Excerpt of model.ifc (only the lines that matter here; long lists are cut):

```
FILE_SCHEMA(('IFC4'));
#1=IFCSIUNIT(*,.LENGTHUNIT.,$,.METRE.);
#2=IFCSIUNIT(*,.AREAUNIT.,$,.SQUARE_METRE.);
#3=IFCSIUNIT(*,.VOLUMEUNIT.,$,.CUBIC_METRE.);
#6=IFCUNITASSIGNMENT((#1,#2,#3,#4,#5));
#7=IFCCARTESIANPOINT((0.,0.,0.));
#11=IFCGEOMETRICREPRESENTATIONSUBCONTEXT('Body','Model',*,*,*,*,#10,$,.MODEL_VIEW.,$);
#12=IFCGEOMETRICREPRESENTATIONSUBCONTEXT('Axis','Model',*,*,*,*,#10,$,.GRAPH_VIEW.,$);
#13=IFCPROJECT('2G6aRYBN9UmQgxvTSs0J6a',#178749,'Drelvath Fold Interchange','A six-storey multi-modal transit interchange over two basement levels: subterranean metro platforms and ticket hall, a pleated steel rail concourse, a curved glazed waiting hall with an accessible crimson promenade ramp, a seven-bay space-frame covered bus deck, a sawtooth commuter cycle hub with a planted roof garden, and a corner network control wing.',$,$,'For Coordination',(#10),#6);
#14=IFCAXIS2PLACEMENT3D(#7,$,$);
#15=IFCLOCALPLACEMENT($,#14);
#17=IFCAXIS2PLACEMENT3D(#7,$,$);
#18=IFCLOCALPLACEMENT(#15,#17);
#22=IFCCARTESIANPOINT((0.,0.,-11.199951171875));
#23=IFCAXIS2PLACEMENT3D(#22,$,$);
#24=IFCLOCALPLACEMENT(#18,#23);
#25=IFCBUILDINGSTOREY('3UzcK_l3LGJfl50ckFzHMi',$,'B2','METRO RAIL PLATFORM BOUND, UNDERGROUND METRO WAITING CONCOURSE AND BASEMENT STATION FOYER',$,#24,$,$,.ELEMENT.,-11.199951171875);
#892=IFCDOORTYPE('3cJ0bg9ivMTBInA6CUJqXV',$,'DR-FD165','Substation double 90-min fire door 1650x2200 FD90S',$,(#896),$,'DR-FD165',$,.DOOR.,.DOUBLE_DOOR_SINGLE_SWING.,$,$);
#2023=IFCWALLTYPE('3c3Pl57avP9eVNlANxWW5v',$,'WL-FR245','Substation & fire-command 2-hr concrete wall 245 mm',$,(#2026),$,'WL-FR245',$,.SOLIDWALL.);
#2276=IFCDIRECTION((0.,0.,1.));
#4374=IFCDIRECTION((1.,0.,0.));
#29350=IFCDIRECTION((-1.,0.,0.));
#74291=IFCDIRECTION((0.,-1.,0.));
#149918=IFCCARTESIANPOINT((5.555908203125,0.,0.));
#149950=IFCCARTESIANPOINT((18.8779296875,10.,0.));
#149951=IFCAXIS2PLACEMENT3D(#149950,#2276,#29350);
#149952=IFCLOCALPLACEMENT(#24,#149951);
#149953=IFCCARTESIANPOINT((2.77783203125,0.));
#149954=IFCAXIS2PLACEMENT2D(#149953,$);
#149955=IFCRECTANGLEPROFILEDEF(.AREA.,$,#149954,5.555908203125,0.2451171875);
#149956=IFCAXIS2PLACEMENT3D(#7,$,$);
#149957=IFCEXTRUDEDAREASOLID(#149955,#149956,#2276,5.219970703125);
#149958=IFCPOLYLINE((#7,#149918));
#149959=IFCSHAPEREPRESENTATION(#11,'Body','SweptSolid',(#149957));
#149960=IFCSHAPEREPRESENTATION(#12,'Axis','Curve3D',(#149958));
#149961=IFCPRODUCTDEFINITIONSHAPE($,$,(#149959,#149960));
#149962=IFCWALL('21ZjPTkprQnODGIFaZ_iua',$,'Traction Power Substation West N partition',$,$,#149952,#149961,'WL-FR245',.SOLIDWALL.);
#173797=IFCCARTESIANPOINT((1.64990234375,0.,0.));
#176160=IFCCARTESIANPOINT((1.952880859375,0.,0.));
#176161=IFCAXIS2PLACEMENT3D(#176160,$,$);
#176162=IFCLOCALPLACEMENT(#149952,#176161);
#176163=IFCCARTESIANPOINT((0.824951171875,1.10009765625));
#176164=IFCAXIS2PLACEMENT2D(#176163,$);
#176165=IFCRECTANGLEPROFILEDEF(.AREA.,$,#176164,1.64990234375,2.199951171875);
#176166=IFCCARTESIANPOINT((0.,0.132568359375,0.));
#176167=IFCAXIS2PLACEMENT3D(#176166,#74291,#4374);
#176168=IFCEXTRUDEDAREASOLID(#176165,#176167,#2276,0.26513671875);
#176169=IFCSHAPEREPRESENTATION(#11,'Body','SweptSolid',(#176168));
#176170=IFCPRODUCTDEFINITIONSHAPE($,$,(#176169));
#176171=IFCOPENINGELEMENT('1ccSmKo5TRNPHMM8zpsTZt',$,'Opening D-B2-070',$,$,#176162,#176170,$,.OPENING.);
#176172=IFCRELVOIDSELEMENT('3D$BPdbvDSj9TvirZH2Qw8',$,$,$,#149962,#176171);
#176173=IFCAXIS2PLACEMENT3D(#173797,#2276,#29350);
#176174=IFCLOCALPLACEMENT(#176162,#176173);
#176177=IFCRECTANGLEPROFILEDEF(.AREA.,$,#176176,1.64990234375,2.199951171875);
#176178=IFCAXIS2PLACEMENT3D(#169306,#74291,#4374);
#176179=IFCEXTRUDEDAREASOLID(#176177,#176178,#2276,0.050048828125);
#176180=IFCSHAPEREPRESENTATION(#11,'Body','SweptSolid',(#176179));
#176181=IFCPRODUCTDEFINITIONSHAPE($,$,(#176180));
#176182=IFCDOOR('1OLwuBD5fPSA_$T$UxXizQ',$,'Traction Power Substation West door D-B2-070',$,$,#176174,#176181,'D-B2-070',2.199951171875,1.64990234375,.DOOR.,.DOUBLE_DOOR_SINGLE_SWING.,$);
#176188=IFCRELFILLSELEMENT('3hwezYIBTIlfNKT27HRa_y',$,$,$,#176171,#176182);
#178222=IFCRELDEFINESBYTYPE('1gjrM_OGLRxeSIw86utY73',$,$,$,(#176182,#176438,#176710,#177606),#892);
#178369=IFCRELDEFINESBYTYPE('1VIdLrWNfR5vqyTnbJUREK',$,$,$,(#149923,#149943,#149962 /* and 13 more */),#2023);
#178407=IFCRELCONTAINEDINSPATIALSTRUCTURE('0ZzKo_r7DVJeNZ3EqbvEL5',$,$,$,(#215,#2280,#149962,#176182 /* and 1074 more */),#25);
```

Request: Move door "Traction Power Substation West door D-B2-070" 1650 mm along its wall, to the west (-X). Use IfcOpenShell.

```python
import ifcopenshell
import ifcopenshell.api.geometry
import ifcopenshell.util.placement

model = ifcopenshell.open("model.ifc")

door = model.by_guid("1OLwuBD5fPSA_$T$UxXizQ")
opening = door.FillsVoids[0].RelatingOpeningElement
wall = opening.VoidsElements[0].RelatingBuildingElement

wall_matrix = ifcopenshell.util.placement.get_local_placement(wall.ObjectPlacement)
shift = wall_matrix[:3, 0] * 1.65
before = ifcopenshell.util.placement.get_local_placement(door.ObjectPlacement)[:3, 3].copy()

# The door is placed relative to its opening, so it follows when the opening moves.
matrix = ifcopenshell.util.placement.get_local_placement(opening.ObjectPlacement)
matrix[:3, 3] += shift
ifcopenshell.api.geometry.edit_object_placement(
    model, product=opening, matrix=matrix, is_si=False, should_transform_children=True
)

after = ifcopenshell.util.placement.get_local_placement(door.ObjectPlacement)[:3, 3]
print("door moved by", (after - before).round(3) + 0.0)

model.write("model_edited.ifc")
```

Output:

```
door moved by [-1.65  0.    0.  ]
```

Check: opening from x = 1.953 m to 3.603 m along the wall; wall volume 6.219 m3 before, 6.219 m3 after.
